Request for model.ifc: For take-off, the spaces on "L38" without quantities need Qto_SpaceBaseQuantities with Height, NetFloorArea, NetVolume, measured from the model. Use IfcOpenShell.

First a look at what the model holds.

```python
import ifcopenshell
import ifcopenshell.util.element
import ifcopenshell.util.unit

model = ifcopenshell.open("model.ifc")
print(model.schema)
for unit_type in ("LENGTHUNIT", "AREAUNIT", "VOLUMEUNIT"):
    print(unit_type, ifcopenshell.util.unit.calculate_unit_scale(model, unit_type))
storey = next(s for s in model.by_type("IfcBuildingStorey") if s.Name == "L38")
spaces = [e for e in ifcopenshell.util.element.get_decomposition(storey) if e.is_a("IfcSpace")]
for e in sorted(spaces, key=lambda e: e.id()):
    print(e.id(), e.is_a(), e.Name, list(ifcopenshell.util.element.get_psets(e, qtos_only=True)), sep=" | ")
```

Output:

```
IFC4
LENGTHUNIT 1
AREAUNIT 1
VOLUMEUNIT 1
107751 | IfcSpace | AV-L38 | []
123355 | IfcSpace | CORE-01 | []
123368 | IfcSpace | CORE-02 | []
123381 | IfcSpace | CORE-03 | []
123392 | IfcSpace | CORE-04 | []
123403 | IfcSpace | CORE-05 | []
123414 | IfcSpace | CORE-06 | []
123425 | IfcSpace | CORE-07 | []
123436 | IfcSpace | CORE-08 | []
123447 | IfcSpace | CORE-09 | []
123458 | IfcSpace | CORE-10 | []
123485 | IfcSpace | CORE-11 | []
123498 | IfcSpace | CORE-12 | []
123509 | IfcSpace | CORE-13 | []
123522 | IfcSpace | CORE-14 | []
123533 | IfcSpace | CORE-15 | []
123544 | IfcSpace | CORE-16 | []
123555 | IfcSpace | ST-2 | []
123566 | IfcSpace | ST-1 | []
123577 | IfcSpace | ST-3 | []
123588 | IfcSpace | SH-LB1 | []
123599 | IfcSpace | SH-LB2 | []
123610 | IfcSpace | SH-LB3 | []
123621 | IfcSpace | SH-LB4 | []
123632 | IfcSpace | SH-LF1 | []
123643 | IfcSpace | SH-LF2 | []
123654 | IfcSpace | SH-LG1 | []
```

```python
import ifcopenshell
import ifcopenshell.api.pset
import ifcopenshell.geom
import ifcopenshell.util.element
import ifcopenshell.util.shape
import ifcopenshell.util.unit

model = ifcopenshell.open("model.ifc")
unit_scale = ifcopenshell.util.unit.calculate_unit_scale(model)
area_scale = ifcopenshell.util.unit.calculate_unit_scale(model, "AREAUNIT")
volume_scale = ifcopenshell.util.unit.calculate_unit_scale(model, "VOLUMEUNIT")
settings = ifcopenshell.geom.settings()

storey = next(s for s in model.by_type("IfcBuildingStorey") if s.Name == "L38")
spaces = [e for e in ifcopenshell.util.element.get_decomposition(storey) if e.is_a("IfcSpace")]

for e in sorted(spaces, key=lambda e: e.id()):
    if ifcopenshell.util.element.get_psets(e, qtos_only=True, should_inherit=False):
        continue
    # Geometry comes back in metres, in the element's own axes.
    shape = ifcopenshell.geom.create_shape(settings, e)
    values = {
        "Height": ifcopenshell.util.shape.get_z(shape.geometry) / unit_scale,
        "NetFloorArea": ifcopenshell.util.shape.get_footprint_area(shape.geometry) / area_scale,
        "NetVolume": ifcopenshell.util.shape.get_volume(shape.geometry) / volume_scale,
    }
    qto = ifcopenshell.api.pset.add_qto(model, product=e, name="Qto_SpaceBaseQuantities")
    ifcopenshell.api.pset.edit_qto(model, qto=qto, properties=values)
    print(e.id(), {k: round(v, 3) for k, v in values.items()})

model.write("model_updated.ifc")
```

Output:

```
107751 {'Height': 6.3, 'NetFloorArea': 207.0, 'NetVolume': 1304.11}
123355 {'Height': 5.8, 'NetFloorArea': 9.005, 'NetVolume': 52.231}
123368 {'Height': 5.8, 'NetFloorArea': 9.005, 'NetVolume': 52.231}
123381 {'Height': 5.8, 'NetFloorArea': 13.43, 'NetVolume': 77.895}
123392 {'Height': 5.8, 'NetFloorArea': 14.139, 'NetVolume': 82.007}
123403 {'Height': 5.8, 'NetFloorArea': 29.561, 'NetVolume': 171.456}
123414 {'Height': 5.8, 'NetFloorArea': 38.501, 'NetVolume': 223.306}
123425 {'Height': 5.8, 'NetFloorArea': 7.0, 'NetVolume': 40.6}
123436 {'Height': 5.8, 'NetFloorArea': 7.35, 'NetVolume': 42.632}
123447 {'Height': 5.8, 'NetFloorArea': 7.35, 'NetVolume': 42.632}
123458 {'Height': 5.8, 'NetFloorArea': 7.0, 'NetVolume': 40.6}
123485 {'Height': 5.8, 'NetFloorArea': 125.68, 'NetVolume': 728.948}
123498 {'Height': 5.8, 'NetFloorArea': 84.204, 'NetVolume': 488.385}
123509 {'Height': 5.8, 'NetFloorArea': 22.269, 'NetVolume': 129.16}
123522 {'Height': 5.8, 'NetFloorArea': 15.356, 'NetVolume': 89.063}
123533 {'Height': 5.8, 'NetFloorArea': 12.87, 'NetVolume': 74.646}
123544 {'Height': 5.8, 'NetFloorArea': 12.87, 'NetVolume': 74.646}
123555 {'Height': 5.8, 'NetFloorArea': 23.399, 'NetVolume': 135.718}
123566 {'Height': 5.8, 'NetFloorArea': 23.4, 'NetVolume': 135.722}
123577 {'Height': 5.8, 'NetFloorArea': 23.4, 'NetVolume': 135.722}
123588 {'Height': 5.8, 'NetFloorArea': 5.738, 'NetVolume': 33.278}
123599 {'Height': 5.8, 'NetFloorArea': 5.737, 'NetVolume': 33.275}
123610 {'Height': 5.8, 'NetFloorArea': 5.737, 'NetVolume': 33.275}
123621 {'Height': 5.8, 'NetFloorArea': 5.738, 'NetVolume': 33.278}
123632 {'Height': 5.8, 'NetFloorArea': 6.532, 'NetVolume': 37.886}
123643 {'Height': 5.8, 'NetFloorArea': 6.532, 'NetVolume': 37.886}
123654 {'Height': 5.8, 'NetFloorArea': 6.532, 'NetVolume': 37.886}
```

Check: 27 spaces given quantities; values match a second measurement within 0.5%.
